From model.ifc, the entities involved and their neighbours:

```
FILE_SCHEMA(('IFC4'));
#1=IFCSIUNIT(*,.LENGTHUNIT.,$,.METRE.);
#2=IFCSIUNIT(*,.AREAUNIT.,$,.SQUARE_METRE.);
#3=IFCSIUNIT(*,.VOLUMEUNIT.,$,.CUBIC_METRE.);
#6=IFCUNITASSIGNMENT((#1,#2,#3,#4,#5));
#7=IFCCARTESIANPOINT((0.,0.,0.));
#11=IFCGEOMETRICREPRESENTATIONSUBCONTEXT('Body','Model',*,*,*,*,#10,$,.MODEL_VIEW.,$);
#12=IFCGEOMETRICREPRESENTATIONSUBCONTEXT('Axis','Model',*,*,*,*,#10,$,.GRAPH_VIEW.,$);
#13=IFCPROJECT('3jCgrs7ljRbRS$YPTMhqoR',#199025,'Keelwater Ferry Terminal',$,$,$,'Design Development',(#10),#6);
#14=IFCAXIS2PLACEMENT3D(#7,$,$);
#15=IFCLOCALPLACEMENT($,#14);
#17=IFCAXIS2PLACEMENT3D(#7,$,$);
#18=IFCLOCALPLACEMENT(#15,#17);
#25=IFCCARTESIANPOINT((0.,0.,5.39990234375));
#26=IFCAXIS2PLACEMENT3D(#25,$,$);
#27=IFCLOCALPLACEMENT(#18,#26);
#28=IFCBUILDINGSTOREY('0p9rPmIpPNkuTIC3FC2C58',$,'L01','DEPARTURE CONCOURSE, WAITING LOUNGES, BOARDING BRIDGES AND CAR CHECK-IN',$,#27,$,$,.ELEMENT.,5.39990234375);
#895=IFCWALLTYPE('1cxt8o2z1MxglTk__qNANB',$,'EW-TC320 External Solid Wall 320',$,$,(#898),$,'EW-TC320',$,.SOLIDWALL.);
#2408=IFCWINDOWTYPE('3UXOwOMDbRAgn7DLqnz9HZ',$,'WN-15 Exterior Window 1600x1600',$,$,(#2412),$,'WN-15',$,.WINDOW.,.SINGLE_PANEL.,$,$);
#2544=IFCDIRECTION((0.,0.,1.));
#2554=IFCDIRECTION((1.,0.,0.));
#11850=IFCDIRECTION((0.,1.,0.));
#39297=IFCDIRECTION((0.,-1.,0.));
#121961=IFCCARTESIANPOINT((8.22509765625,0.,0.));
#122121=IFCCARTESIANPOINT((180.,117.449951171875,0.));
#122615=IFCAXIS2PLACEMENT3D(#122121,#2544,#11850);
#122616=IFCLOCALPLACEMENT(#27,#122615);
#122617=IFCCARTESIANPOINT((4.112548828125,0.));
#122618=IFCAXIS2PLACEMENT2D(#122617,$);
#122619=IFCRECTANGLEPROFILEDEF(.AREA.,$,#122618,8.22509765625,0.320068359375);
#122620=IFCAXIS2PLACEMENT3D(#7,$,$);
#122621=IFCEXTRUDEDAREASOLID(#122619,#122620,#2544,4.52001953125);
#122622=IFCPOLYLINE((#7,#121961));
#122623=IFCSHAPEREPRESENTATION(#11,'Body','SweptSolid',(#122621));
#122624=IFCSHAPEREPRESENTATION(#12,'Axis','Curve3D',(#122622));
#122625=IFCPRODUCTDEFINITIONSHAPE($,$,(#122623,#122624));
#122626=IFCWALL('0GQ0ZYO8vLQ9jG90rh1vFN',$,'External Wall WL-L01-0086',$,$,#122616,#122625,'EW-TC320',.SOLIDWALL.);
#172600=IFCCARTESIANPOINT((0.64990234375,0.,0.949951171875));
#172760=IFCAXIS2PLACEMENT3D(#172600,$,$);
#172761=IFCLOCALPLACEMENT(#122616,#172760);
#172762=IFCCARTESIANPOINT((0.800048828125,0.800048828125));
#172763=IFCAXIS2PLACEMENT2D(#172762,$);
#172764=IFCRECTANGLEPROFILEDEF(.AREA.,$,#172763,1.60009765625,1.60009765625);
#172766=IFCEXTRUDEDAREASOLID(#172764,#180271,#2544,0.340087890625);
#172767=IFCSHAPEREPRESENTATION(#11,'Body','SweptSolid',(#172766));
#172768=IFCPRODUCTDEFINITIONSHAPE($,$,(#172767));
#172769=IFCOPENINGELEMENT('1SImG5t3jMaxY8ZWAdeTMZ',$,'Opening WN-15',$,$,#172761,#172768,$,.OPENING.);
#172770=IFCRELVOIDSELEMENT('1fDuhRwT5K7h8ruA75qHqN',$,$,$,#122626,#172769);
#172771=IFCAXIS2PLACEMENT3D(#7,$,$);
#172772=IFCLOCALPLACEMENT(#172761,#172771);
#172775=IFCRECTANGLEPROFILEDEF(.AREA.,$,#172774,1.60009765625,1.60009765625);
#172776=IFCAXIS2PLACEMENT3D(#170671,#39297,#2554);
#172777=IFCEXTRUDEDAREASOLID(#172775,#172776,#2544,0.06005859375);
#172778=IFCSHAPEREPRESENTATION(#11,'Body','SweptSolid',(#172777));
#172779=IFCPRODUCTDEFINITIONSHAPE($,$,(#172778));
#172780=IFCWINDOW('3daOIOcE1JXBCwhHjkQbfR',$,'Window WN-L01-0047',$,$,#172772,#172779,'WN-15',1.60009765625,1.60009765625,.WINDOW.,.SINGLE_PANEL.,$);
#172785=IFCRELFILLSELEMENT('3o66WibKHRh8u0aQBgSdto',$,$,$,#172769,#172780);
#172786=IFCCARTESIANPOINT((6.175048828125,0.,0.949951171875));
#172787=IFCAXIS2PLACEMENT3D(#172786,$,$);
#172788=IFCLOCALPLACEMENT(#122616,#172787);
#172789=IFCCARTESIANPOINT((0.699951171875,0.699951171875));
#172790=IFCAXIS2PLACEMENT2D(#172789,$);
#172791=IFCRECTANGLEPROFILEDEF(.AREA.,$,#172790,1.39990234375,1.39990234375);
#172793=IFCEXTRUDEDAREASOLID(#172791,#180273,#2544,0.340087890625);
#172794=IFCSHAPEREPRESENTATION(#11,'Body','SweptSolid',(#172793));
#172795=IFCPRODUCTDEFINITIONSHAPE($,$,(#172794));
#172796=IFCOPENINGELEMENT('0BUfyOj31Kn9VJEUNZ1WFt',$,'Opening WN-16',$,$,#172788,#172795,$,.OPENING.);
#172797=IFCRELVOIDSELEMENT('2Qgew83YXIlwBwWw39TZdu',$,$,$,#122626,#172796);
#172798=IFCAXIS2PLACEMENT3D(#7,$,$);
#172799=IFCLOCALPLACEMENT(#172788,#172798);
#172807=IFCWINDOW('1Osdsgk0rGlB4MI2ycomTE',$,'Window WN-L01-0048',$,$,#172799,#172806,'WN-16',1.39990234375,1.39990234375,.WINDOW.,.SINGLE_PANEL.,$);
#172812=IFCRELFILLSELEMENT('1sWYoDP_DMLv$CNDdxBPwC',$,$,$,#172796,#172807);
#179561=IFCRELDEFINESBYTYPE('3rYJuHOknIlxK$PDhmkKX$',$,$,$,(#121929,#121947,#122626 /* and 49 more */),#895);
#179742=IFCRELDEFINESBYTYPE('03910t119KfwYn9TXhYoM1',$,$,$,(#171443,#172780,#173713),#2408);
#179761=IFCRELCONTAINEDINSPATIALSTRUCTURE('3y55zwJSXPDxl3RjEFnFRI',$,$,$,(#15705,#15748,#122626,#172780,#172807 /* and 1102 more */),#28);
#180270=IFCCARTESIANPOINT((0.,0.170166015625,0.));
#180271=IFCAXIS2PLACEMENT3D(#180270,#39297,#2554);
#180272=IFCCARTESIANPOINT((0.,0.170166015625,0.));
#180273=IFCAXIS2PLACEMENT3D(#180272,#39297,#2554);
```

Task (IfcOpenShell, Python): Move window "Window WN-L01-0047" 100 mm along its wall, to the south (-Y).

```python
import ifcopenshell
import ifcopenshell.api.geometry
import ifcopenshell.util.placement
import ifcopenshell.util.unit

model = ifcopenshell.open("model.ifc")
unit_scale = ifcopenshell.util.unit.calculate_unit_scale(model)

window = model.by_id(172780)
opening = window.FillsVoids[0].RelatingOpeningElement
wall = opening.VoidsElements[0].RelatingBuildingElement

wall_matrix = ifcopenshell.util.placement.get_local_placement(wall.ObjectPlacement)
shift = wall_matrix[:3, 0] * -0.1 / unit_scale
before = ifcopenshell.util.placement.get_local_placement(window.ObjectPlacement)[:3, 3].copy()

# The window is placed relative to its opening, so it follows when the opening moves.
matrix = ifcopenshell.util.placement.get_local_placement(opening.ObjectPlacement)
matrix[:3, 3] += shift
ifcopenshell.api.geometry.edit_object_placement(
    model, product=opening, matrix=matrix, is_si=False, should_transform_children=True
)

after = ifcopenshell.util.placement.get_local_placement(window.ObjectPlacement)[:3, 3]
print("window moved by", (after - before).round(3) + 0.0)

model.write("model_rev.ifc")
```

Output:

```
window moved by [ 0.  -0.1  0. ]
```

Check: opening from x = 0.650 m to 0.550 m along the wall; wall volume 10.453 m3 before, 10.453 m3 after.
